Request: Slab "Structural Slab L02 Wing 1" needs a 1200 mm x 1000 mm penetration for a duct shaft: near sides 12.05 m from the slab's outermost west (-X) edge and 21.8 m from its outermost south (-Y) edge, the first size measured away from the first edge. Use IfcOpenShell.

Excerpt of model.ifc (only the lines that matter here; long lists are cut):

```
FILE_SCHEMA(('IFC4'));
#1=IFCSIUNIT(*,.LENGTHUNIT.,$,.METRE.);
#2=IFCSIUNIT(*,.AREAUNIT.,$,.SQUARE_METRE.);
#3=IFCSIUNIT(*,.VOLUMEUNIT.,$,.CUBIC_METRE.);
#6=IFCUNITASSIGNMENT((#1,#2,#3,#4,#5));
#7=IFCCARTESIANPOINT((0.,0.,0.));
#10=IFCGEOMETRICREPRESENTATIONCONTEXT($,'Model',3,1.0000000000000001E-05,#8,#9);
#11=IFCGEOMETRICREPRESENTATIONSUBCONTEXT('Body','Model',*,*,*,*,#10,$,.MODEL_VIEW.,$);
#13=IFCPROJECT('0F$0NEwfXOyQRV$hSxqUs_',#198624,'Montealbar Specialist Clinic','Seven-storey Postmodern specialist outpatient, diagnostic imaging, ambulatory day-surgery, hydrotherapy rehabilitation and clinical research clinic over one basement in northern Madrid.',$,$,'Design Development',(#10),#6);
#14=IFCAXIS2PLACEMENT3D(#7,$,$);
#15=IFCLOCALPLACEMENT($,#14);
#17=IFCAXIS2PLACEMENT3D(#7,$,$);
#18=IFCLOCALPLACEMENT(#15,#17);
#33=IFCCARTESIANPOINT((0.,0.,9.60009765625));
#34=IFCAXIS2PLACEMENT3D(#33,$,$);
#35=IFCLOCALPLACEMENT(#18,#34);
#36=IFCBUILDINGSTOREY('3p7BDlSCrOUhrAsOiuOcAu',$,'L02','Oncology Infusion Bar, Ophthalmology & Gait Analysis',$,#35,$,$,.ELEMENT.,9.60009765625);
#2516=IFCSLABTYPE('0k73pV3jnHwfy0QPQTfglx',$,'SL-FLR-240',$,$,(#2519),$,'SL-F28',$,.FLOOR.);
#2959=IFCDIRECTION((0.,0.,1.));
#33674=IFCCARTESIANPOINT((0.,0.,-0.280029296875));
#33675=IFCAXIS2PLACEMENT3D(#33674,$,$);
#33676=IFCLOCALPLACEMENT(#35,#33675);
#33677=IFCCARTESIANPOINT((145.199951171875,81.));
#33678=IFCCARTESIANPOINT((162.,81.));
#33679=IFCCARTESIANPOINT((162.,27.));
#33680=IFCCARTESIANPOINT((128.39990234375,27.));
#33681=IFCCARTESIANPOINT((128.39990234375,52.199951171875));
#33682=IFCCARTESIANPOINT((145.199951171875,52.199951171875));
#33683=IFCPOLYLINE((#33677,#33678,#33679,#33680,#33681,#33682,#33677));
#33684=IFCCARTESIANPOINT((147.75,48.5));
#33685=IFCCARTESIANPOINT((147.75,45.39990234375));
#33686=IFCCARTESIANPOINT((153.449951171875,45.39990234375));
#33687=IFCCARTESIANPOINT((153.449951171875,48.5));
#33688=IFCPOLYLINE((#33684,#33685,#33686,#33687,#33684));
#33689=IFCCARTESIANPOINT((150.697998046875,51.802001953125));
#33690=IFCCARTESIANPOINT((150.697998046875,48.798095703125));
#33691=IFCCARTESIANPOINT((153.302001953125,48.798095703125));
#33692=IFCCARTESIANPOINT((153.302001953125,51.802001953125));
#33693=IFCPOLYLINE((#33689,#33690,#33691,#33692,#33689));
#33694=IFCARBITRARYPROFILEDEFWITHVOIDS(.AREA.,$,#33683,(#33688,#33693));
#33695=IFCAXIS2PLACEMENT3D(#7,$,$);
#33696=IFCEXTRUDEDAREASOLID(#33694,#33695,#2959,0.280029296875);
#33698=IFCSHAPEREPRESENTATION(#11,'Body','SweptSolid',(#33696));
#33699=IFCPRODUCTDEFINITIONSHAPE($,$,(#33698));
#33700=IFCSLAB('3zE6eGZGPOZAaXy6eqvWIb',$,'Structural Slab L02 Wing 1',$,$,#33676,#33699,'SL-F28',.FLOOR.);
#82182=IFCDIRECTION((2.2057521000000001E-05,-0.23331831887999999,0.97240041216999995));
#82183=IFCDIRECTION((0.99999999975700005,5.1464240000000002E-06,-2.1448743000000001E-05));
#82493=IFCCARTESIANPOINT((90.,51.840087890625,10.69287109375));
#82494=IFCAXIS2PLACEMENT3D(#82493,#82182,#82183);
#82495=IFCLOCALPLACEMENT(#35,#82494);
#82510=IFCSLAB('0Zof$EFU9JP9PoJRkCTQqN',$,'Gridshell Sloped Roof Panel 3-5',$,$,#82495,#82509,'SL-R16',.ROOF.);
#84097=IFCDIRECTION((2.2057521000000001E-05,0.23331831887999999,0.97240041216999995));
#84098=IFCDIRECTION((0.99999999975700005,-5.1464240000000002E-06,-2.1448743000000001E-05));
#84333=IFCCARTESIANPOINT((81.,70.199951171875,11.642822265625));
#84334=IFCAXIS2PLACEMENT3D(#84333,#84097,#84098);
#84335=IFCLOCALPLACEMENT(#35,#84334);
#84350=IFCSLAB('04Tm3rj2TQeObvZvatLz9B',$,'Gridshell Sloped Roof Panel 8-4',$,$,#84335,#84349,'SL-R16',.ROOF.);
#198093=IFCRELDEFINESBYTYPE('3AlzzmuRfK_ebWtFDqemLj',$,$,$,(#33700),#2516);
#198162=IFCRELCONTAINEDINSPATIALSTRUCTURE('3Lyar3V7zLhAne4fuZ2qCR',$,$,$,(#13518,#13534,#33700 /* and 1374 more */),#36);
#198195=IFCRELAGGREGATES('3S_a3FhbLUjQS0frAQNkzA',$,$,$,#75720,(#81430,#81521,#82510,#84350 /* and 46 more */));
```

```python
import numpy as np
import ifcopenshell
import ifcopenshell.api.feature
import ifcopenshell.api.geometry
import ifcopenshell.api.root
import ifcopenshell.geom
import ifcopenshell.util.placement
import ifcopenshell.util.representation
import ifcopenshell.util.shape
import ifcopenshell.util.unit

model = ifcopenshell.open("model.ifc")
unit_scale = ifcopenshell.util.unit.calculate_unit_scale(model)
settings = ifcopenshell.geom.settings()


def volume(element):
    """Net volume in cubic metres, openings subtracted."""
    shape = ifcopenshell.geom.create_shape(settings, element)
    return ifcopenshell.util.shape.get_volume(shape.geometry)


slab = model.by_id(33700)
before = volume(slab)

# Extent in the slab's own axes, in metres. The edges named are its -X and -Y sides.
slab_shape = ifcopenshell.geom.create_shape(settings, slab)
vertices = ifcopenshell.util.shape.get_vertices(slab_shape.geometry)
x_min, y_min, bottom = vertices.min(axis=0)
top = vertices[:, 2].max()

opening = ifcopenshell.api.root.create_entity(model, ifc_class="IfcOpeningElement", name="Duct shaft opening", predefined_type="OPENING")
context = ifcopenshell.util.representation.get_context(model, "Model", "Body", "MODEL_VIEW")
width, depth = 1.2, 1
outline = [(0.0, 0.0), (width, 0.0), (width, depth), (0.0, depth), (0.0, 0.0)]
# Overshoot both faces by 50 mm so the cut is clean.
shape = ifcopenshell.api.geometry.add_slab_representation(
    model, context=context, depth=top - bottom + 0.1, polyline=outline
)
ifcopenshell.api.geometry.assign_representation(model, product=opening, representation=shape)

matrix = ifcopenshell.util.placement.get_local_placement(slab.ObjectPlacement)
matrix[:, 3] = matrix @ np.append(np.array([x_min + 12.05, y_min + 21.8, bottom - 0.05]) / unit_scale, 1.0)
ifcopenshell.api.geometry.edit_object_placement(model, product=opening, matrix=matrix, is_si=False)
ifcopenshell.api.feature.add_feature(model, feature=opening, element=slab)

after = volume(slab)

print(f"slab volume {before:.3f} -> {after:.3f} m3")

model.write("model_updated.ifc")
```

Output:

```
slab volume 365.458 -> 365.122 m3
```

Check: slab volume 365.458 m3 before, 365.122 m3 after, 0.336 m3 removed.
